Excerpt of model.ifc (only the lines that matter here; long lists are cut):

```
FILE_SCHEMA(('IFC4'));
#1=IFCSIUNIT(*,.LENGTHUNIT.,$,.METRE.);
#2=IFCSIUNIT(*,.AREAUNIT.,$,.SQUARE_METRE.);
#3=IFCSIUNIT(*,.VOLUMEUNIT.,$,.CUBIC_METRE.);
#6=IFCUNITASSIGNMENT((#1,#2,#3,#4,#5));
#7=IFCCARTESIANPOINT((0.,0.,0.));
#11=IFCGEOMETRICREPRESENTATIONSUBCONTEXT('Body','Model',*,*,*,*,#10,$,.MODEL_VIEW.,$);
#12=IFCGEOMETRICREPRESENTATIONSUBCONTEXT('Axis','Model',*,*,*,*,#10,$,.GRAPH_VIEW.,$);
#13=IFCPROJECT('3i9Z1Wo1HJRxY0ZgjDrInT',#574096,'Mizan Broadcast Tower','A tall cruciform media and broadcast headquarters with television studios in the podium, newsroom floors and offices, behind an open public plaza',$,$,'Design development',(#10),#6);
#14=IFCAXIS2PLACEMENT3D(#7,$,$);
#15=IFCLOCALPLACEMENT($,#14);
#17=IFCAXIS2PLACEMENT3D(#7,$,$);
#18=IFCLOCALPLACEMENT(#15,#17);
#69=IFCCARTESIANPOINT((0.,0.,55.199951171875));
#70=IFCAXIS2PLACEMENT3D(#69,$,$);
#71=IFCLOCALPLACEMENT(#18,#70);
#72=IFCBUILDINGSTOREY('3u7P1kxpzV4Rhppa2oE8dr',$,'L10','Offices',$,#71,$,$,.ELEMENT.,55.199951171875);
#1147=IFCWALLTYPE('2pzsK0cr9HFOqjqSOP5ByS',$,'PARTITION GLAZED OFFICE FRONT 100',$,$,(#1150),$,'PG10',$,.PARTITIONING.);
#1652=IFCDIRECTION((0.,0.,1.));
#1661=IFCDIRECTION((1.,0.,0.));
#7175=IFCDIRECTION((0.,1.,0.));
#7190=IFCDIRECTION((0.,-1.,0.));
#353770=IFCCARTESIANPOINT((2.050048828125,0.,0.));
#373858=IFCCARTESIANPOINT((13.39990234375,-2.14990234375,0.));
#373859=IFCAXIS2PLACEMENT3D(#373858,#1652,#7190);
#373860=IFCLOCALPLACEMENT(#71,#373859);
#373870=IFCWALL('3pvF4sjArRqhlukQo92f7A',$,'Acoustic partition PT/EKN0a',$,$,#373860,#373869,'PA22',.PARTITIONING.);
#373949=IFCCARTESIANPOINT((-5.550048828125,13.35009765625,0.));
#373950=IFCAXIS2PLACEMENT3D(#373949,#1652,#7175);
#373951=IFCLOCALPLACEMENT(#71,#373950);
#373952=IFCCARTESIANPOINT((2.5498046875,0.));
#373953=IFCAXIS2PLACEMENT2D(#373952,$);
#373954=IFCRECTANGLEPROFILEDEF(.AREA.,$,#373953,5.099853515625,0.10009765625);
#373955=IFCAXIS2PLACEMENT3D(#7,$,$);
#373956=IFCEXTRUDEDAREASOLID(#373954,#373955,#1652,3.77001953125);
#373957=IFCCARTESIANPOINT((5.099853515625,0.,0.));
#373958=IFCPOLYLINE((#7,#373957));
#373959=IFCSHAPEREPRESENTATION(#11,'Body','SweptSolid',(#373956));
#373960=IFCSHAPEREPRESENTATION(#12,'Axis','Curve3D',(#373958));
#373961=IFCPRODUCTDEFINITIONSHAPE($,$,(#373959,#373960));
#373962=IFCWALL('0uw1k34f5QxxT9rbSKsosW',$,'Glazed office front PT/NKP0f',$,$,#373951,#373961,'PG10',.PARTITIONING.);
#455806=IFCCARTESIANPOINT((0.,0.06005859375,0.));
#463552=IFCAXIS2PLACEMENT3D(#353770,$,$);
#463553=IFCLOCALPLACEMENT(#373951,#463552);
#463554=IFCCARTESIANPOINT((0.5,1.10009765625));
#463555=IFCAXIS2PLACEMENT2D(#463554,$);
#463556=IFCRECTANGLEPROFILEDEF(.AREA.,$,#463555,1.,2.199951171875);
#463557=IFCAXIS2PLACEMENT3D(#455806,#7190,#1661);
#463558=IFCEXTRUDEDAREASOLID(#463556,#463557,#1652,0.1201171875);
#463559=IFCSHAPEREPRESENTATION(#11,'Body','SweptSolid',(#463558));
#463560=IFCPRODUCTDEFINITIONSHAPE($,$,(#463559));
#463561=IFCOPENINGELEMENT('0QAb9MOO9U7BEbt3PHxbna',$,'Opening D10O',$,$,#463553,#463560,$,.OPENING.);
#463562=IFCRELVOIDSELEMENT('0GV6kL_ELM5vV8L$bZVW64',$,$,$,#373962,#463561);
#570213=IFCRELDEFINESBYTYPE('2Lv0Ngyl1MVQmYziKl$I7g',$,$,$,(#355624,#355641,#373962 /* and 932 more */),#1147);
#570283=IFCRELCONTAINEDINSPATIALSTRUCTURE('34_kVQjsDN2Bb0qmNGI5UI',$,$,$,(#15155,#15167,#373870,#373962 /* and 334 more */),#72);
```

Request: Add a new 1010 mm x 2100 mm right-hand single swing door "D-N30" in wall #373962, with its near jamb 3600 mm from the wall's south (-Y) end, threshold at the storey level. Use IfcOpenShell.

```python
import numpy as np
import ifcopenshell
import ifcopenshell.api.feature
import ifcopenshell.api.geometry
import ifcopenshell.api.root
import ifcopenshell.api.spatial
import ifcopenshell.geom
import ifcopenshell.util.element
import ifcopenshell.util.placement
import ifcopenshell.util.representation
import ifcopenshell.util.shape
import ifcopenshell.util.unit

model = ifcopenshell.open("model.ifc")
unit_scale = ifcopenshell.util.unit.calculate_unit_scale(model)
settings = ifcopenshell.geom.settings()


def volume(element):
    """Net volume in cubic metres, openings subtracted."""
    shape = ifcopenshell.geom.create_shape(settings, element)
    return ifcopenshell.util.shape.get_volume(shape.geometry)


wall = model.by_guid("0uw1k34f5QxxT9rbSKsosW")
storey = ifcopenshell.util.element.get_container(wall, ifc_class="IfcBuildingStorey")
context = ifcopenshell.util.representation.get_context(model, "Model", "Body", "MODEL_VIEW")
before = volume(wall)

width, height, from_end, sill = 1.01, 2.1, 3.6, 0.0  # metres

# The wall runs along its own X axis, and the end named is its -X end.
wall_shape = ifcopenshell.geom.create_shape(settings, wall)
x, y, z = ifcopenshell.util.shape.get_vertices(wall_shape.geometry).T
start = x.min() + from_end
face, thickness = float(y.min()), float(y.max() - y.min())
wall_matrix = ifcopenshell.util.placement.get_local_placement(wall.ObjectPlacement)
level = ifcopenshell.util.placement.get_local_placement(storey.ObjectPlacement)[2, 3]


def in_wall(x, y):
    """Placement at x, y metres in the wall's axes, at sill height."""
    matrix = wall_matrix.copy()
    matrix[:, 3] = wall_matrix @ np.array([x / unit_scale, y / unit_scale, 0.0, 1.0])
    matrix[2, 3] = level + sill / unit_scale
    return matrix


# Opening: a box that overshoots both wall faces by 50 mm.
opening = ifcopenshell.api.root.create_entity(model, ifc_class="IfcOpeningElement", predefined_type="OPENING")
box = ifcopenshell.api.geometry.add_wall_representation(
    model, context=context, length=width, height=height, thickness=thickness + 0.1
)
ifcopenshell.api.geometry.assign_representation(model, product=opening, representation=box)
ifcopenshell.api.geometry.edit_object_placement(model, product=opening, matrix=in_wall(start, face - 0.05), is_si=False)
ifcopenshell.api.feature.add_feature(model, feature=opening, element=wall)

door = ifcopenshell.api.root.create_entity(model, ifc_class="IfcDoor", name="D-N30", predefined_type="DOOR")
door.OverallWidth, door.OverallHeight = width / unit_scale, height / unit_scale
door.OperationType = "SINGLE_SWING_RIGHT"
body = ifcopenshell.api.geometry.add_door_representation(
    model,
    context=context,
    overall_width=door.OverallWidth,
    overall_height=door.OverallHeight,
    operation_type="SINGLE_SWING_RIGHT",
    lining_properties={"LiningDepth": thickness / unit_scale, "ThresholdDepth": thickness / unit_scale},
)
ifcopenshell.api.geometry.assign_representation(model, product=door, representation=body)
ifcopenshell.api.spatial.assign_container(model, products=[door], relating_structure=storey)
ifcopenshell.api.feature.add_filling(model, opening=opening, element=door)

# The lining spans the wall, so the door starts at the wall face.
ifcopenshell.api.geometry.edit_object_placement(model, product=door, matrix=in_wall(start, face), is_si=False)

after = volume(wall)

print(f"wall volume {before:.3f} -> {after:.3f} m3")

model.write("model_updated.ifc")
```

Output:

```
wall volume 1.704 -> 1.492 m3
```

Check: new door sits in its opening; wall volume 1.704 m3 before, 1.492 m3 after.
